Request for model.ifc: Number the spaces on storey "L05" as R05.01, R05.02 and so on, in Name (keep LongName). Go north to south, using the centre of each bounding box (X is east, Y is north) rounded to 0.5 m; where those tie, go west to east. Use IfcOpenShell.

First a look at what the model holds.

```python
import ifcopenshell
import ifcopenshell.util.element
import ifcopenshell.util.placement

model = ifcopenshell.open("model.ifc")
print(model.schema)
storey = next(s for s in model.by_type("IfcBuildingStorey") if s.Name == "L05")
spaces = [e for e in ifcopenshell.util.element.get_decomposition(storey) if e.is_a("IfcSpace")]
for e in sorted(spaces, key=lambda e: e.id()):
    origin = ifcopenshell.util.placement.get_local_placement(e.ObjectPlacement)[:3, 3]
    print(e.id(), e.Name, e.LongName, origin.round(2) + 0.0, sep=" | ")
```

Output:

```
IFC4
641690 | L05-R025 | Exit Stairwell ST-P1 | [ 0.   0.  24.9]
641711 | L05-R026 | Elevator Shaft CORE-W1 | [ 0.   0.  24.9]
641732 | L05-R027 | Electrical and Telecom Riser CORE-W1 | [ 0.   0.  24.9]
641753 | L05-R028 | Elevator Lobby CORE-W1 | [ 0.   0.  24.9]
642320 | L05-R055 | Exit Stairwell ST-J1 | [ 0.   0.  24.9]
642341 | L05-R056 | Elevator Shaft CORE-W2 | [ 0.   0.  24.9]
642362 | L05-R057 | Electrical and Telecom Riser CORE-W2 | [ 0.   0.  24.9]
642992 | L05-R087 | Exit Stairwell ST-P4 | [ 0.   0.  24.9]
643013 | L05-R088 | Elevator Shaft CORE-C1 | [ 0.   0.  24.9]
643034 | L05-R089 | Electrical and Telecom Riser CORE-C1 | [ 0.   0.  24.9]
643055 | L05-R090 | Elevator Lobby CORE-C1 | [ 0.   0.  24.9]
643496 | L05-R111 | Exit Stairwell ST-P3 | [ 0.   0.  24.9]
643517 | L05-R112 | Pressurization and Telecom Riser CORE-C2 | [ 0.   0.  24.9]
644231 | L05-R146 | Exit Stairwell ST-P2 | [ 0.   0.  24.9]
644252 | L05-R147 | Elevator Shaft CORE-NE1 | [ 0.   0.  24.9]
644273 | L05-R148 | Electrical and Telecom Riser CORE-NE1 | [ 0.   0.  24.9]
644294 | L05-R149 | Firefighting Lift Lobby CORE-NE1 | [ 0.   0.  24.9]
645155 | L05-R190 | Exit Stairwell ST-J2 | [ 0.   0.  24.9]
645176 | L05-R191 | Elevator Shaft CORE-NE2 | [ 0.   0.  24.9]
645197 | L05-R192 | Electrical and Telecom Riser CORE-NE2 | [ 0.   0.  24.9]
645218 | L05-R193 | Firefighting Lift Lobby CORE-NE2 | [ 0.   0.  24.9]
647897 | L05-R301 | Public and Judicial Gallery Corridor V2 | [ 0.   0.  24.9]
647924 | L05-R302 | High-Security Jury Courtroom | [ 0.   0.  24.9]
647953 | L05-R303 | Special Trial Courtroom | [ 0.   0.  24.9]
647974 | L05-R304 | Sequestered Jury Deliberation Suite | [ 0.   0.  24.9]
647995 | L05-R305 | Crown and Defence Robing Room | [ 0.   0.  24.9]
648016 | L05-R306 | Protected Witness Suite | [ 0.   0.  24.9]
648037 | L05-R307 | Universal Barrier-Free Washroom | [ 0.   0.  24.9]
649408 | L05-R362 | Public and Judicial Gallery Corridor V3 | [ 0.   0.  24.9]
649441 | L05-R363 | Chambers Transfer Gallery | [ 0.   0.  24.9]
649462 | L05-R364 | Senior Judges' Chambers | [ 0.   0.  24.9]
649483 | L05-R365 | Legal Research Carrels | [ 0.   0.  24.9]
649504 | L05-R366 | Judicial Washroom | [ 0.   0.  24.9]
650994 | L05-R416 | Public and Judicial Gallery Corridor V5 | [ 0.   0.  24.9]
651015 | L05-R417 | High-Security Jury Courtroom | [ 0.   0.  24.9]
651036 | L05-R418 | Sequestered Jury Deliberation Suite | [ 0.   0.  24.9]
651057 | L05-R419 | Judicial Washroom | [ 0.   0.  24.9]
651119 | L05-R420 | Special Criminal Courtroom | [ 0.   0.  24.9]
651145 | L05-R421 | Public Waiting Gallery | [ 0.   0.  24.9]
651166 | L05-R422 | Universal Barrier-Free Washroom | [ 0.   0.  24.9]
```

```python
import ifcopenshell
import ifcopenshell.geom
import ifcopenshell.util.element
import ifcopenshell.util.shape

model = ifcopenshell.open("model.ifc")
settings = ifcopenshell.geom.settings()
settings.set("use-world-coords", True)


def centre(element):
    shape = ifcopenshell.geom.create_shape(settings, element)
    return ifcopenshell.util.shape.get_bbox_centroid(shape.geometry)


storey = next(s for s in model.by_type("IfcBuildingStorey") if s.Name == "L05")
spaces = [e for e in ifcopenshell.util.element.get_decomposition(storey) if e.is_a("IfcSpace")]

# Insertion points can sit at a corner or the storey origin, so sort by the geometry (in metres).
centres = {e: centre(e) for e in spaces}
spaces.sort(key=lambda e: (-round(centres[e][1] / 0.5), centres[e][0]))

for i, e in enumerate(spaces, start=1):
    number = f"R05.{i:02d}"
    e.Name = number
    print(e.id(), number)

model.write("model_updated.ifc")
```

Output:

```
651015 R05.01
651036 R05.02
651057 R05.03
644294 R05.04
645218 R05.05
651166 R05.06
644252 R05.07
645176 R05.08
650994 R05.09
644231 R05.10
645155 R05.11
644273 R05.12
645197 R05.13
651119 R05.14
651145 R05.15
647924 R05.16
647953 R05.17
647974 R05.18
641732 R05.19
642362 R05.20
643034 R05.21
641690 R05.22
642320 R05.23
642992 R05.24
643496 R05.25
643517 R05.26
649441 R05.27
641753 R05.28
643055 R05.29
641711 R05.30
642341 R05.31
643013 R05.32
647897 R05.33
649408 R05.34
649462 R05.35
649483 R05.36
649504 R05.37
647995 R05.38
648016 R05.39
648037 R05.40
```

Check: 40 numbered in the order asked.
